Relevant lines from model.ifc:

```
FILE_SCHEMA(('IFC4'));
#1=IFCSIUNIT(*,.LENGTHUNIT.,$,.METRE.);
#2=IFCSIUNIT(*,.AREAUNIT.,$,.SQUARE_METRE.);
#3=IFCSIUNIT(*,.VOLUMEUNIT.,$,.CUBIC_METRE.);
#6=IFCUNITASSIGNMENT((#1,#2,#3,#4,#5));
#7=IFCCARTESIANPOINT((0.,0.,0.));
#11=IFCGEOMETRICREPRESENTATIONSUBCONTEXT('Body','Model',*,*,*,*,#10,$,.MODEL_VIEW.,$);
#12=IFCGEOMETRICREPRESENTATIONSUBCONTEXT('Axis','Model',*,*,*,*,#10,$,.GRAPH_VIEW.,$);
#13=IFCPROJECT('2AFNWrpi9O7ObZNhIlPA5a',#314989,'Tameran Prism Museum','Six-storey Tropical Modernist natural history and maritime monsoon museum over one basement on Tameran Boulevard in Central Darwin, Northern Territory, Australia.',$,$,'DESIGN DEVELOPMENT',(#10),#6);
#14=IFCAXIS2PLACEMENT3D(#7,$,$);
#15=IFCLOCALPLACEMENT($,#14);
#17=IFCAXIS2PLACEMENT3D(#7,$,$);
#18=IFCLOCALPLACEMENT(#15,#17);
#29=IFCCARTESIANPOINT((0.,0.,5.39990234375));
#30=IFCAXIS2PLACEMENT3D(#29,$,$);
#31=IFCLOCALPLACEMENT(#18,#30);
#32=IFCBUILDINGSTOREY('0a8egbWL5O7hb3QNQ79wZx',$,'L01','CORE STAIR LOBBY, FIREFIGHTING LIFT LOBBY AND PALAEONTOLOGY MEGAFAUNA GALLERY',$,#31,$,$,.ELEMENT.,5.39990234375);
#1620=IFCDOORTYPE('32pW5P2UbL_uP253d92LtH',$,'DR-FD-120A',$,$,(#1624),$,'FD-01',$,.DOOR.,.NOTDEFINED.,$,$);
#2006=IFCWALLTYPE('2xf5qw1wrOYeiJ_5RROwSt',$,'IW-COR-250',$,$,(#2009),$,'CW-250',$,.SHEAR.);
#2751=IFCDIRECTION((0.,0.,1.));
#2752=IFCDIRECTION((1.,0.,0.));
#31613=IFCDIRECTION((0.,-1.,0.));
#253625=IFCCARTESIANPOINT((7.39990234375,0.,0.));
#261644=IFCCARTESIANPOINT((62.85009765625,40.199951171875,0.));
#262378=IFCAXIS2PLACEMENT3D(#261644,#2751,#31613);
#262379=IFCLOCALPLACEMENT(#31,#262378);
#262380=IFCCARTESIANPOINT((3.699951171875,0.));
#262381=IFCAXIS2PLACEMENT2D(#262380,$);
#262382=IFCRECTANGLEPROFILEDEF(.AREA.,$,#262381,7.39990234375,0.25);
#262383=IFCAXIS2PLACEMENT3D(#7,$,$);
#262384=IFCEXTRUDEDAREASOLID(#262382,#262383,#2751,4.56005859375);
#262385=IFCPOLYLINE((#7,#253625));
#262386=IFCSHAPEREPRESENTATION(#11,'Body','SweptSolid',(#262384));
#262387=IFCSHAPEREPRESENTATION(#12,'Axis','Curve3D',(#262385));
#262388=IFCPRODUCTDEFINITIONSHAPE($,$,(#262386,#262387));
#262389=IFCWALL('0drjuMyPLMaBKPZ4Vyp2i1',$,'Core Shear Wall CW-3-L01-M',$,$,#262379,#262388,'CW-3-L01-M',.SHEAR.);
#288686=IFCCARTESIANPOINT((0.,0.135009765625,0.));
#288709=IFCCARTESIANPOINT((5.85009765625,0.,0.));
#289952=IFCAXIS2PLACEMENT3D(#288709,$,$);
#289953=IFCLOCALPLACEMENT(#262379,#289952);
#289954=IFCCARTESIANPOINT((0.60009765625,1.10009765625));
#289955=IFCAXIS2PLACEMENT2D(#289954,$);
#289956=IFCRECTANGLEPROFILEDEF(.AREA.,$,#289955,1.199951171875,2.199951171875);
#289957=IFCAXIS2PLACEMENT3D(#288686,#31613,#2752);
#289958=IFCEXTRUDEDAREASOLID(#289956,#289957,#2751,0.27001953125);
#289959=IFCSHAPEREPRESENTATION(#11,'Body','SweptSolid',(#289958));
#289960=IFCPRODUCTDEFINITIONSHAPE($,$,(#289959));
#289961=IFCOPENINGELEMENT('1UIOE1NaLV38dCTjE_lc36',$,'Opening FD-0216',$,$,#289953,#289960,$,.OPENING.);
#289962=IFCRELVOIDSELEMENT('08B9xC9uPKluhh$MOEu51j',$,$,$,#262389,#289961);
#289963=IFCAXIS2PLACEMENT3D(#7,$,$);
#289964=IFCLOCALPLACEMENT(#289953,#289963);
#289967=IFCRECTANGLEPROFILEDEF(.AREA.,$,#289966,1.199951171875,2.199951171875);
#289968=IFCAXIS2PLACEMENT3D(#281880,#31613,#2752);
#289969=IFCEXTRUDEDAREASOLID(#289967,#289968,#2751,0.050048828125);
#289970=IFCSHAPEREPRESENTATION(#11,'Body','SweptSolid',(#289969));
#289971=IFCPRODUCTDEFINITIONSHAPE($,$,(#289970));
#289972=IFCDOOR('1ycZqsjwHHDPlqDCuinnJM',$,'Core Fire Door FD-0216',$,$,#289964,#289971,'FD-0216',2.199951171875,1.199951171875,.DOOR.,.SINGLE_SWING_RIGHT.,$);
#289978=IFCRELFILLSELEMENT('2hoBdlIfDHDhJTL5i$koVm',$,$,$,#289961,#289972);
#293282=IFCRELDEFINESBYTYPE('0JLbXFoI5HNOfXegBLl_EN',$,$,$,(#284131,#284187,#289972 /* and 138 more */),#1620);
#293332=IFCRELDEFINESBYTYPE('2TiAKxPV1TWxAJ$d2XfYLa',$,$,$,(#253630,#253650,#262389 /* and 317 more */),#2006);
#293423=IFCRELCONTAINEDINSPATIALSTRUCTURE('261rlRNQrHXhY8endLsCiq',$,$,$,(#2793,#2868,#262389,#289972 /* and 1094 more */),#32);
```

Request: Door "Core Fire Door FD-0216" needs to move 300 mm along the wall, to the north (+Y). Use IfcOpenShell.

```python
import ifcopenshell
import ifcopenshell.api.geometry
import ifcopenshell.util.placement
import ifcopenshell.util.unit

model = ifcopenshell.open("model.ifc")
unit_scale = ifcopenshell.util.unit.calculate_unit_scale(model)

door = model.by_guid("1ycZqsjwHHDPlqDCuinnJM")
opening = door.FillsVoids[0].RelatingOpeningElement
wall = opening.VoidsElements[0].RelatingBuildingElement

wall_matrix = ifcopenshell.util.placement.get_local_placement(wall.ObjectPlacement)
shift = wall_matrix[:3, 0] * -0.3 / unit_scale
before = ifcopenshell.util.placement.get_local_placement(door.ObjectPlacement)[:3, 3].copy()

# The door is placed relative to its opening, so it follows when the opening moves.
matrix = ifcopenshell.util.placement.get_local_placement(opening.ObjectPlacement)
matrix[:3, 3] += shift
ifcopenshell.api.geometry.edit_object_placement(
    model, product=opening, matrix=matrix, is_si=False, should_transform_children=True
)

after = ifcopenshell.util.placement.get_local_placement(door.ObjectPlacement)[:3, 3]
print("door moved by", (after - before).round(3) + 0.0)

model.write("model_edited.ifc")
```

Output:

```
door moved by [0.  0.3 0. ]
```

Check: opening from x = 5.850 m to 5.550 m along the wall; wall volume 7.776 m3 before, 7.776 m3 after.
